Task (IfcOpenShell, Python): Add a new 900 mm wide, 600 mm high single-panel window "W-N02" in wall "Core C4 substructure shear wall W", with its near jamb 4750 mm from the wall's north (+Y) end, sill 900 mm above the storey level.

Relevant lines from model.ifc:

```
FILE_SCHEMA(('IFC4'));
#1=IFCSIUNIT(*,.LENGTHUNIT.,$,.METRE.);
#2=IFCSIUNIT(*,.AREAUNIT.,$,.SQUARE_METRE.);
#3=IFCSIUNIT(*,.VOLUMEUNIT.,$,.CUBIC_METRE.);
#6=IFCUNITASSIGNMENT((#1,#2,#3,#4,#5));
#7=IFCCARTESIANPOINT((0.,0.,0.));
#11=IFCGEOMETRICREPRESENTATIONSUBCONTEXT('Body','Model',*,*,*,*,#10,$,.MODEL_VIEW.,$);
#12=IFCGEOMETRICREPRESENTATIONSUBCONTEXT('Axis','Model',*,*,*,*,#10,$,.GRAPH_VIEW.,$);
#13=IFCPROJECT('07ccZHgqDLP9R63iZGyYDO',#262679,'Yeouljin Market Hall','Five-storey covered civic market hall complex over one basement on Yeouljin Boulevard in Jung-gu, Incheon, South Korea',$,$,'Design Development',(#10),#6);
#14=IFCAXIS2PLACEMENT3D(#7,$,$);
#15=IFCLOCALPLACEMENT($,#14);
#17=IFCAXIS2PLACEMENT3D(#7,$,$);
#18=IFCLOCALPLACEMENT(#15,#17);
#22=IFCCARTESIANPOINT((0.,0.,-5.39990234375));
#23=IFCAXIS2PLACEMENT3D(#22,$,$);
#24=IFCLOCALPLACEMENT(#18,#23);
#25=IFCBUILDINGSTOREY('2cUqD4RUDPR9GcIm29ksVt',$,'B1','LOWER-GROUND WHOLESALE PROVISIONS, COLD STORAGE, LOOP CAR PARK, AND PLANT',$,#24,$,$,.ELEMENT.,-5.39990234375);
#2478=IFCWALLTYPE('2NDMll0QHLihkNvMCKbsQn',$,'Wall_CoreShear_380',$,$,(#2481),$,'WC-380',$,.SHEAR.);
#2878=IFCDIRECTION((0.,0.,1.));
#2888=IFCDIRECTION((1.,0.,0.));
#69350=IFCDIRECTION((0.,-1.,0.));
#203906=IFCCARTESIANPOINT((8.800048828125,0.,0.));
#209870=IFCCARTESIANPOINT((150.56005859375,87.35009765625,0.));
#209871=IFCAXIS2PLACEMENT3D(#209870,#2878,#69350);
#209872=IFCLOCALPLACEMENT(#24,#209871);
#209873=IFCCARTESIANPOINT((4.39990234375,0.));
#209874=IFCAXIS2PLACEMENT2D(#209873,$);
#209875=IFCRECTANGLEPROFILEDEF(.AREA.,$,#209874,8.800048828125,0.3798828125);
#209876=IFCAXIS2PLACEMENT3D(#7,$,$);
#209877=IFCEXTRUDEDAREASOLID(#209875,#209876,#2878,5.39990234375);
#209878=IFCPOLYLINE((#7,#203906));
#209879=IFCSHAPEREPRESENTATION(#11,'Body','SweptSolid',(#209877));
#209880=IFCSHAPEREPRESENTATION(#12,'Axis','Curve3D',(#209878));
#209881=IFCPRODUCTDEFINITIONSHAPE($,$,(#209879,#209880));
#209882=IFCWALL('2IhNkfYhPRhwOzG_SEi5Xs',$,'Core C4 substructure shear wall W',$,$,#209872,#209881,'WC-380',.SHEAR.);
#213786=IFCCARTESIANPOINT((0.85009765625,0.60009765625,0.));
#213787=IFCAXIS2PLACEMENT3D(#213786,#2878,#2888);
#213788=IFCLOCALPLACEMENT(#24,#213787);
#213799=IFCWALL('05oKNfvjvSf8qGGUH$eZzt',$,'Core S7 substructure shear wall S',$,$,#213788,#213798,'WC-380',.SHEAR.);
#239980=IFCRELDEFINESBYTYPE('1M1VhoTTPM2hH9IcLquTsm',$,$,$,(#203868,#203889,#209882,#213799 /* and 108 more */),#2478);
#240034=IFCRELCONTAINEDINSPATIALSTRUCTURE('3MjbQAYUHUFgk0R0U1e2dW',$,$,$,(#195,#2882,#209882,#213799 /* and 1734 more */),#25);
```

```python
import numpy as np
import ifcopenshell
import ifcopenshell.api.feature
import ifcopenshell.api.geometry
import ifcopenshell.api.root
import ifcopenshell.api.spatial
import ifcopenshell.geom
import ifcopenshell.util.element
import ifcopenshell.util.placement
import ifcopenshell.util.representation
import ifcopenshell.util.shape
import ifcopenshell.util.unit

model = ifcopenshell.open("model.ifc")
unit_scale = ifcopenshell.util.unit.calculate_unit_scale(model)
settings = ifcopenshell.geom.settings()


def volume(element):
    """Net volume in cubic metres, openings subtracted."""
    shape = ifcopenshell.geom.create_shape(settings, element)
    return ifcopenshell.util.shape.get_volume(shape.geometry)


wall = model.by_id(209882)
storey = ifcopenshell.util.element.get_container(wall, ifc_class="IfcBuildingStorey")
context = ifcopenshell.util.representation.get_context(model, "Model", "Body", "MODEL_VIEW")
before = volume(wall)

width, height, from_end, sill = 0.9, 0.6, 4.75, 0.9  # metres

# The wall runs along its own X axis, and the end named is its -X end.
wall_shape = ifcopenshell.geom.create_shape(settings, wall)
x, y, z = ifcopenshell.util.shape.get_vertices(wall_shape.geometry).T
start = x.min() + from_end
face, thickness = float(y.min()), float(y.max() - y.min())
wall_matrix = ifcopenshell.util.placement.get_local_placement(wall.ObjectPlacement)
level = ifcopenshell.util.placement.get_local_placement(storey.ObjectPlacement)[2, 3]


def in_wall(x, y):
    """Placement at x, y metres in the wall's axes, at sill height."""
    matrix = wall_matrix.copy()
    matrix[:, 3] = wall_matrix @ np.array([x / unit_scale, y / unit_scale, 0.0, 1.0])
    matrix[2, 3] = level + sill / unit_scale
    return matrix


# Opening: a box that overshoots both wall faces by 50 mm.
opening = ifcopenshell.api.root.create_entity(model, ifc_class="IfcOpeningElement", predefined_type="OPENING")
box = ifcopenshell.api.geometry.add_wall_representation(
    model, context=context, length=width, height=height, thickness=thickness + 0.1
)
ifcopenshell.api.geometry.assign_representation(model, product=opening, representation=box)
ifcopenshell.api.geometry.edit_object_placement(model, product=opening, matrix=in_wall(start, face - 0.05), is_si=False)
ifcopenshell.api.feature.add_feature(model, feature=opening, element=wall)

window = ifcopenshell.api.root.create_entity(model, ifc_class="IfcWindow", name="W-N02", predefined_type="WINDOW")
window.OverallWidth, window.OverallHeight = width / unit_scale, height / unit_scale
window.PartitioningType = "SINGLE_PANEL"
body = ifcopenshell.api.geometry.add_window_representation(
    model,
    context=context,
    overall_width=window.OverallWidth,
    overall_height=window.OverallHeight,
    partition_type="SINGLE_PANEL",
)
ifcopenshell.api.geometry.assign_representation(model, product=window, representation=body)
ifcopenshell.api.spatial.assign_container(model, products=[window], relating_structure=storey)
ifcopenshell.api.feature.add_filling(model, opening=opening, element=window)

# Centre the window in the wall's thickness.
ifcopenshell.api.geometry.edit_object_placement(model, product=window, matrix=in_wall(start, face), is_si=False)
window_shape = ifcopenshell.geom.create_shape(settings, window)
depth = ifcopenshell.util.shape.get_vertices(window_shape.geometry)[:, 1]
offset = face + thickness / 2 - (depth.min() + depth.max()) / 2
ifcopenshell.api.geometry.edit_object_placement(model, product=window, matrix=in_wall(start, offset), is_si=False)

after = volume(wall)

print(f"wall volume {before:.3f} -> {after:.3f} m3")

model.write("model_edited.ifc")
```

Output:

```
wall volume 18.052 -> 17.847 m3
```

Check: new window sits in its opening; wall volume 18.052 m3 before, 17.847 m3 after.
